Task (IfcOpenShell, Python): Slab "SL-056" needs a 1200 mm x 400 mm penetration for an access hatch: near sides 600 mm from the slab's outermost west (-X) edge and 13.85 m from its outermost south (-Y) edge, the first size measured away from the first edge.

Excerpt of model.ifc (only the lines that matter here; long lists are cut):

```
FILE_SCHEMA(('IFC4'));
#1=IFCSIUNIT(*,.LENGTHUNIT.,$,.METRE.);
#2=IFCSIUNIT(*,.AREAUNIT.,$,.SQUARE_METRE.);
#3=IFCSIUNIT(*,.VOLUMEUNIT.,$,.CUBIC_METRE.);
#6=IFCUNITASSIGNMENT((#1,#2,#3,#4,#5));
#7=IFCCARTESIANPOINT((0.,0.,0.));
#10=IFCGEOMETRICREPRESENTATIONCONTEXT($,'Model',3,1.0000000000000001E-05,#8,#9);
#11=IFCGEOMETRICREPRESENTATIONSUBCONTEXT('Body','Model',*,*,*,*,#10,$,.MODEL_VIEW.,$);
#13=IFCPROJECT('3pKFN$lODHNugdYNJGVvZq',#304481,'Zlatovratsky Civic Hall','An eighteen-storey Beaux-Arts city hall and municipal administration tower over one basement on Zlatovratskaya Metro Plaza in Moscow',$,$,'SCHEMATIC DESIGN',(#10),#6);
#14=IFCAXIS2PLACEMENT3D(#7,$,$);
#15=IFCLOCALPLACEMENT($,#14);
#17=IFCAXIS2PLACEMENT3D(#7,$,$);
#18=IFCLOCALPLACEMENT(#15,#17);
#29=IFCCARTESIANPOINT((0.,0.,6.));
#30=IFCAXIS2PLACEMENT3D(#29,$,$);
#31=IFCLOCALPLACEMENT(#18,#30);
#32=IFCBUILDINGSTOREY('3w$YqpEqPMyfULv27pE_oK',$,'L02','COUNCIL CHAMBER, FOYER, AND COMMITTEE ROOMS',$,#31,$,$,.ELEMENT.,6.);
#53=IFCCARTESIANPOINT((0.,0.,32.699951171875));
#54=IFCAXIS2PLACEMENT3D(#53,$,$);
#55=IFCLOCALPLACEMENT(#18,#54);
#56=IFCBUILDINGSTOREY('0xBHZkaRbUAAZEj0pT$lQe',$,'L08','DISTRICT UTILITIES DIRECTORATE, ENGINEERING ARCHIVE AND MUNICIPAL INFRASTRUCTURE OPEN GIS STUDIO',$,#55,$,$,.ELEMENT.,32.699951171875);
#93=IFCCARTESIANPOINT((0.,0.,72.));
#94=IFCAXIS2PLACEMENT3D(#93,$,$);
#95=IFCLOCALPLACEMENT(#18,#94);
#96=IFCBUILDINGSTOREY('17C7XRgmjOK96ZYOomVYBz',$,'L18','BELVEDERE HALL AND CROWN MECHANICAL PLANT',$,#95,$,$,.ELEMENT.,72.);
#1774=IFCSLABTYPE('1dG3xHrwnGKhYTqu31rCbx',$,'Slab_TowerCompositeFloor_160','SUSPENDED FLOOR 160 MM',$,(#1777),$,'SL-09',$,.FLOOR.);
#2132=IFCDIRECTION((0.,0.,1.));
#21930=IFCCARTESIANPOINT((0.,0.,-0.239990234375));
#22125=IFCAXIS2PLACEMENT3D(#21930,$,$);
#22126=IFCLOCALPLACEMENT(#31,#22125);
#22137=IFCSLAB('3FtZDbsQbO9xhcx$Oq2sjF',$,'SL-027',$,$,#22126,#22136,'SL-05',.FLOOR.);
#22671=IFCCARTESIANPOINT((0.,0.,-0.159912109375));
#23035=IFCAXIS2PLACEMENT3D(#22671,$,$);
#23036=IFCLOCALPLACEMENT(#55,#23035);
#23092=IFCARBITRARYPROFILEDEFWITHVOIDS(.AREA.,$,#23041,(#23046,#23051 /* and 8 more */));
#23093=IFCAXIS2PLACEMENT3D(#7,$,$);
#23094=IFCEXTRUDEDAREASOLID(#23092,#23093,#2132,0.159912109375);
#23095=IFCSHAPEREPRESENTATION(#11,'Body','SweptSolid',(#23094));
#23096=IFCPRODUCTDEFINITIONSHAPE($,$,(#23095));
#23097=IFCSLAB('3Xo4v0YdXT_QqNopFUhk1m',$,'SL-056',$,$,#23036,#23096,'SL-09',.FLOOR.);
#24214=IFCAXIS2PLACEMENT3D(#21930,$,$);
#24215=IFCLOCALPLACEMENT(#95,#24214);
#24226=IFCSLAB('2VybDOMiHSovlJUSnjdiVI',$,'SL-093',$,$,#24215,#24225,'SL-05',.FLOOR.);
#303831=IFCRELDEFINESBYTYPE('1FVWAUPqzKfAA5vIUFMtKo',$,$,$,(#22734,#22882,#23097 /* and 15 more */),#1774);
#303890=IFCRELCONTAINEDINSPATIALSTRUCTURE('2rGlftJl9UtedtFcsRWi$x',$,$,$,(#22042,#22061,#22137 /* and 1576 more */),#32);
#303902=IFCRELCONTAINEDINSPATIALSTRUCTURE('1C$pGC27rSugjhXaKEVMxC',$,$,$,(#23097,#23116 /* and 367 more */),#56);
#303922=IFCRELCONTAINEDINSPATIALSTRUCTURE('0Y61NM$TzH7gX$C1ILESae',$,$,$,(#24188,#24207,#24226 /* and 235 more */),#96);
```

```python
import numpy as np
import ifcopenshell
import ifcopenshell.api.feature
import ifcopenshell.api.geometry
import ifcopenshell.api.root
import ifcopenshell.geom
import ifcopenshell.util.placement
import ifcopenshell.util.representation
import ifcopenshell.util.shape
import ifcopenshell.util.unit

model = ifcopenshell.open("model.ifc")
unit_scale = ifcopenshell.util.unit.calculate_unit_scale(model)
settings = ifcopenshell.geom.settings()


def volume(element):
    """Net volume in cubic metres, openings subtracted."""
    shape = ifcopenshell.geom.create_shape(settings, element)
    return ifcopenshell.util.shape.get_volume(shape.geometry)


slab = model.by_guid("3Xo4v0YdXT_QqNopFUhk1m")
before = volume(slab)

# Extent in the slab's own axes, in metres. The edges named are its -X and -Y sides.
slab_shape = ifcopenshell.geom.create_shape(settings, slab)
vertices = ifcopenshell.util.shape.get_vertices(slab_shape.geometry)
x_min, y_min, bottom = vertices.min(axis=0)
top = vertices[:, 2].max()

opening = ifcopenshell.api.root.create_entity(model, ifc_class="IfcOpeningElement", name="Access hatch opening", predefined_type="OPENING")
context = ifcopenshell.util.representation.get_context(model, "Model", "Body", "MODEL_VIEW")
width, depth = 1.2, 0.4
outline = [(0.0, 0.0), (width, 0.0), (width, depth), (0.0, depth), (0.0, 0.0)]
# Overshoot both faces by 50 mm so the cut is clean.
shape = ifcopenshell.api.geometry.add_slab_representation(
    model, context=context, depth=top - bottom + 0.1, polyline=outline
)
ifcopenshell.api.geometry.assign_representation(model, product=opening, representation=shape)

matrix = ifcopenshell.util.placement.get_local_placement(slab.ObjectPlacement)
matrix[:, 3] = matrix @ np.append(np.array([x_min + 0.6, y_min + 13.85, bottom - 0.05]) / unit_scale, 1.0)
ifcopenshell.api.geometry.edit_object_placement(model, product=opening, matrix=matrix, is_si=False)
ifcopenshell.api.feature.add_feature(model, feature=opening, element=slab)

after = volume(slab)

print(f"slab volume {before:.3f} -> {after:.3f} m3")

model.write("model-out.ifc")
```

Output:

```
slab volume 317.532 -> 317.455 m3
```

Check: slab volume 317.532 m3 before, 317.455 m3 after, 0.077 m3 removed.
